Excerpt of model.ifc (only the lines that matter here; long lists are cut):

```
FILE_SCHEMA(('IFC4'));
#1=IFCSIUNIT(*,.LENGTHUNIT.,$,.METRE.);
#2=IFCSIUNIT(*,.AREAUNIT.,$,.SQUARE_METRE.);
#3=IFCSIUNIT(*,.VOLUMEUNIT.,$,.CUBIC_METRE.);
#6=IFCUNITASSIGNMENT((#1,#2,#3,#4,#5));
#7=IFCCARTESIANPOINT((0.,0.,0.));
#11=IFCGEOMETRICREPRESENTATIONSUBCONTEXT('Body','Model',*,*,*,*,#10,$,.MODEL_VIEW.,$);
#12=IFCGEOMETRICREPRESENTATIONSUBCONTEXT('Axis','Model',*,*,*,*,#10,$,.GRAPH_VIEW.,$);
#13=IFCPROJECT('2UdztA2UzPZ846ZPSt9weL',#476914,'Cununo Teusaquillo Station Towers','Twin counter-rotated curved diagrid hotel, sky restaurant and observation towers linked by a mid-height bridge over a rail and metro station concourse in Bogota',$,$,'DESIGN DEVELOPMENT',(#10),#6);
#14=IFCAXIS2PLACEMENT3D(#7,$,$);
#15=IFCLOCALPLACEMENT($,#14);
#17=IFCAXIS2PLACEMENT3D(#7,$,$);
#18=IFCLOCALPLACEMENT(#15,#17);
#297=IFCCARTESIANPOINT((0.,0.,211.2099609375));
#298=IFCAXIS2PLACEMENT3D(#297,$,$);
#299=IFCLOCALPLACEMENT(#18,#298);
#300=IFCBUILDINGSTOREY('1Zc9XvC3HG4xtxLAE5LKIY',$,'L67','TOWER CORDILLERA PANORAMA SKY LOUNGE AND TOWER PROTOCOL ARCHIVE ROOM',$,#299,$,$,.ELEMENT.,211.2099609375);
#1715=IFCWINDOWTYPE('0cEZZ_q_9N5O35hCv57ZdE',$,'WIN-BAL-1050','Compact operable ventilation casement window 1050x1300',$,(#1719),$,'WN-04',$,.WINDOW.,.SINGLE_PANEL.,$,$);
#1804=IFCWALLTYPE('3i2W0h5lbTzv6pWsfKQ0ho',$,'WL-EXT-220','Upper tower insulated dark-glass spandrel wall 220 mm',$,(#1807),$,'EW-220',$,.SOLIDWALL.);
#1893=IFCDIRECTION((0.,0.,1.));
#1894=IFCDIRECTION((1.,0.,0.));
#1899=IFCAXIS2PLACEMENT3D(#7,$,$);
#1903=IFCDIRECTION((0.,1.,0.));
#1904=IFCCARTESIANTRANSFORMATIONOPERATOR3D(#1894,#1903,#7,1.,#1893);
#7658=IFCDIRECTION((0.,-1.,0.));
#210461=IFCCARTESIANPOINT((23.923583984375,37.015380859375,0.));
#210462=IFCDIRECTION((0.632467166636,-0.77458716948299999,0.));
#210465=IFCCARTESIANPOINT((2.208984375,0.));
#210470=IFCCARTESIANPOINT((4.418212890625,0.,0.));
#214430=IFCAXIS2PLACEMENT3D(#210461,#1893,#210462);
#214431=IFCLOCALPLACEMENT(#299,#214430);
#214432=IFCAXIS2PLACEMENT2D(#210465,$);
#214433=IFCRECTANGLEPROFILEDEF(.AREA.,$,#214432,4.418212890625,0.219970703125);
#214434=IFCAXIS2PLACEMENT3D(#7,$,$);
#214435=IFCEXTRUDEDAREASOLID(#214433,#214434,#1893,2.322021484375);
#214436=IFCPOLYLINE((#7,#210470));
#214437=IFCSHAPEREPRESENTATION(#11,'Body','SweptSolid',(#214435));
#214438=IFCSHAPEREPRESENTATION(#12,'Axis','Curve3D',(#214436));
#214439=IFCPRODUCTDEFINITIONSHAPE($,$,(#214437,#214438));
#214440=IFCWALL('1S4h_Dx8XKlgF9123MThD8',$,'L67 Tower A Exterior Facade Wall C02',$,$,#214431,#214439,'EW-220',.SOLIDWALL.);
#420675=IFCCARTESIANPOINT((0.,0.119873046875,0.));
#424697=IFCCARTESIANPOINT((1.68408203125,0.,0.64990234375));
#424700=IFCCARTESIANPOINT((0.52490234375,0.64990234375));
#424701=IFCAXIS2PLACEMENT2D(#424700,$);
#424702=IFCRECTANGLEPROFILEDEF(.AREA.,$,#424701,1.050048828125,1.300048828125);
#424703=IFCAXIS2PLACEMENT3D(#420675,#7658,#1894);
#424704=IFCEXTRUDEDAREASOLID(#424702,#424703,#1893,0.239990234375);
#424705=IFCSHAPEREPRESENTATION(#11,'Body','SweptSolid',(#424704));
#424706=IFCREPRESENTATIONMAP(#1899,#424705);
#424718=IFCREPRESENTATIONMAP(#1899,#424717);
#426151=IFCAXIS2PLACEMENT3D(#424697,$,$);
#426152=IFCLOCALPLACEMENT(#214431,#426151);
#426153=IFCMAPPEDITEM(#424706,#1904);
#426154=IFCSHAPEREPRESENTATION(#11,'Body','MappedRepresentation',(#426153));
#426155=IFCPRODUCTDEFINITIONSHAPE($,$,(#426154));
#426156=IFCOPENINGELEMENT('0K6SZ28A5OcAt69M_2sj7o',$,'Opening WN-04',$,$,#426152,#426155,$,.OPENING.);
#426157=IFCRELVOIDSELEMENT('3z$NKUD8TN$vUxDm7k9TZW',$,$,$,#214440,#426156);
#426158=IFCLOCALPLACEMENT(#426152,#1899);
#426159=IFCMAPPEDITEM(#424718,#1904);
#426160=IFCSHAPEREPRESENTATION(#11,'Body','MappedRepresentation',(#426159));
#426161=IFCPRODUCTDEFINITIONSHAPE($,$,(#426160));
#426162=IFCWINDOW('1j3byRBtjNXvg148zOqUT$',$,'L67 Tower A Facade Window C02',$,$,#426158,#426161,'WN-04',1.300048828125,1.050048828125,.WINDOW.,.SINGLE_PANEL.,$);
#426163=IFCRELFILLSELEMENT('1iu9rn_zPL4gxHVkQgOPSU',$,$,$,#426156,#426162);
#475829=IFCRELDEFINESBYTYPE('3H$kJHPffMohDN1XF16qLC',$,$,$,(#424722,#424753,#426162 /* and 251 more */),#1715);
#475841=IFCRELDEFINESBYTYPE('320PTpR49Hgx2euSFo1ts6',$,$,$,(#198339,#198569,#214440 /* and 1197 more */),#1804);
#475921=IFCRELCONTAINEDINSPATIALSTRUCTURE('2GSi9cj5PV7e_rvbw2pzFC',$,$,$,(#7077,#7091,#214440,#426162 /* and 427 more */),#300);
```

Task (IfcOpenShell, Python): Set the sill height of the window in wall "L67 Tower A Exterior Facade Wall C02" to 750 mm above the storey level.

```python
import numpy as np
import ifcopenshell
import ifcopenshell.api.geometry
import ifcopenshell.geom
import ifcopenshell.util.element
import ifcopenshell.util.placement
import ifcopenshell.util.shape
import ifcopenshell.util.unit

model = ifcopenshell.open("model.ifc")
unit_scale = ifcopenshell.util.unit.calculate_unit_scale(model)

window = model.by_guid("1j3byRBtjNXvg148zOqUT$")
opening = window.FillsVoids[0].RelatingOpeningElement
storey = ifcopenshell.util.element.get_container(window, ifc_class="IfcBuildingStorey")
level = ifcopenshell.util.placement.get_local_placement(storey.ObjectPlacement)[2, 3]

# The opening's origin need not be at the sill, so measure its lowest point.
shape = ifcopenshell.geom.create_shape(ifcopenshell.geom.settings(), opening)
bottom = ifcopenshell.util.shape.get_shape_bottom_elevation(shape, shape.geometry) / unit_scale
dz = level + 0.75 / unit_scale - bottom

shift = np.array([0.0, 0.0, dz])
# The window is placed relative to its opening, so it follows when the opening moves.
matrix = ifcopenshell.util.placement.get_local_placement(opening.ObjectPlacement)
matrix[:3, 3] += shift
ifcopenshell.api.geometry.edit_object_placement(
    model, product=opening, matrix=matrix, is_si=False, should_transform_children=True
)

print(f"moved by {dz * unit_scale:+.3f} m")

model.write("model_rev.ifc")
```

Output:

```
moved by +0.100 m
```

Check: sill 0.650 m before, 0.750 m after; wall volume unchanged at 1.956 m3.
